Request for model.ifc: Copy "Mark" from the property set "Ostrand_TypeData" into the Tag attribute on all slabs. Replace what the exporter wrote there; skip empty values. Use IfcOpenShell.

First a look at what the model holds.

```python
import ifcopenshell
import ifcopenshell.util.element

model = ifcopenshell.open("model.ifc")
print(model.schema)
slabs = model.by_type("IfcSlab")
print(len(slabs), "slabs")
for e in slabs[:8]:
    source = ifcopenshell.util.element.get_pset(e, "Ostrand_TypeData", "Mark")
    target = e.Tag
    print(e.id(), repr(source), repr(target), sep=" | ")
```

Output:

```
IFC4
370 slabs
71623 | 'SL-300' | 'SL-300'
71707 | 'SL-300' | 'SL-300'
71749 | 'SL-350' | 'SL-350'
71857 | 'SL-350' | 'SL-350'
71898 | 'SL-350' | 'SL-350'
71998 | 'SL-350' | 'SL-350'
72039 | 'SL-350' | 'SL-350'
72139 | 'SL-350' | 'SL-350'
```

```python
import ifcopenshell
import ifcopenshell.util.element

model = ifcopenshell.open("model.ifc")

count = 0
for e in model.by_type("IfcSlab"):
    value = ifcopenshell.util.element.get_pset(e, "Ostrand_TypeData", "Mark")
    current = e.Tag
    if not value or not value.strip() or current == value:
        continue
    e.Tag = value
    count += 1

print(count, "slabs updated")

model.write("model_edited.ifc")
```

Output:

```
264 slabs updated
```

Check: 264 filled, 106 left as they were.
